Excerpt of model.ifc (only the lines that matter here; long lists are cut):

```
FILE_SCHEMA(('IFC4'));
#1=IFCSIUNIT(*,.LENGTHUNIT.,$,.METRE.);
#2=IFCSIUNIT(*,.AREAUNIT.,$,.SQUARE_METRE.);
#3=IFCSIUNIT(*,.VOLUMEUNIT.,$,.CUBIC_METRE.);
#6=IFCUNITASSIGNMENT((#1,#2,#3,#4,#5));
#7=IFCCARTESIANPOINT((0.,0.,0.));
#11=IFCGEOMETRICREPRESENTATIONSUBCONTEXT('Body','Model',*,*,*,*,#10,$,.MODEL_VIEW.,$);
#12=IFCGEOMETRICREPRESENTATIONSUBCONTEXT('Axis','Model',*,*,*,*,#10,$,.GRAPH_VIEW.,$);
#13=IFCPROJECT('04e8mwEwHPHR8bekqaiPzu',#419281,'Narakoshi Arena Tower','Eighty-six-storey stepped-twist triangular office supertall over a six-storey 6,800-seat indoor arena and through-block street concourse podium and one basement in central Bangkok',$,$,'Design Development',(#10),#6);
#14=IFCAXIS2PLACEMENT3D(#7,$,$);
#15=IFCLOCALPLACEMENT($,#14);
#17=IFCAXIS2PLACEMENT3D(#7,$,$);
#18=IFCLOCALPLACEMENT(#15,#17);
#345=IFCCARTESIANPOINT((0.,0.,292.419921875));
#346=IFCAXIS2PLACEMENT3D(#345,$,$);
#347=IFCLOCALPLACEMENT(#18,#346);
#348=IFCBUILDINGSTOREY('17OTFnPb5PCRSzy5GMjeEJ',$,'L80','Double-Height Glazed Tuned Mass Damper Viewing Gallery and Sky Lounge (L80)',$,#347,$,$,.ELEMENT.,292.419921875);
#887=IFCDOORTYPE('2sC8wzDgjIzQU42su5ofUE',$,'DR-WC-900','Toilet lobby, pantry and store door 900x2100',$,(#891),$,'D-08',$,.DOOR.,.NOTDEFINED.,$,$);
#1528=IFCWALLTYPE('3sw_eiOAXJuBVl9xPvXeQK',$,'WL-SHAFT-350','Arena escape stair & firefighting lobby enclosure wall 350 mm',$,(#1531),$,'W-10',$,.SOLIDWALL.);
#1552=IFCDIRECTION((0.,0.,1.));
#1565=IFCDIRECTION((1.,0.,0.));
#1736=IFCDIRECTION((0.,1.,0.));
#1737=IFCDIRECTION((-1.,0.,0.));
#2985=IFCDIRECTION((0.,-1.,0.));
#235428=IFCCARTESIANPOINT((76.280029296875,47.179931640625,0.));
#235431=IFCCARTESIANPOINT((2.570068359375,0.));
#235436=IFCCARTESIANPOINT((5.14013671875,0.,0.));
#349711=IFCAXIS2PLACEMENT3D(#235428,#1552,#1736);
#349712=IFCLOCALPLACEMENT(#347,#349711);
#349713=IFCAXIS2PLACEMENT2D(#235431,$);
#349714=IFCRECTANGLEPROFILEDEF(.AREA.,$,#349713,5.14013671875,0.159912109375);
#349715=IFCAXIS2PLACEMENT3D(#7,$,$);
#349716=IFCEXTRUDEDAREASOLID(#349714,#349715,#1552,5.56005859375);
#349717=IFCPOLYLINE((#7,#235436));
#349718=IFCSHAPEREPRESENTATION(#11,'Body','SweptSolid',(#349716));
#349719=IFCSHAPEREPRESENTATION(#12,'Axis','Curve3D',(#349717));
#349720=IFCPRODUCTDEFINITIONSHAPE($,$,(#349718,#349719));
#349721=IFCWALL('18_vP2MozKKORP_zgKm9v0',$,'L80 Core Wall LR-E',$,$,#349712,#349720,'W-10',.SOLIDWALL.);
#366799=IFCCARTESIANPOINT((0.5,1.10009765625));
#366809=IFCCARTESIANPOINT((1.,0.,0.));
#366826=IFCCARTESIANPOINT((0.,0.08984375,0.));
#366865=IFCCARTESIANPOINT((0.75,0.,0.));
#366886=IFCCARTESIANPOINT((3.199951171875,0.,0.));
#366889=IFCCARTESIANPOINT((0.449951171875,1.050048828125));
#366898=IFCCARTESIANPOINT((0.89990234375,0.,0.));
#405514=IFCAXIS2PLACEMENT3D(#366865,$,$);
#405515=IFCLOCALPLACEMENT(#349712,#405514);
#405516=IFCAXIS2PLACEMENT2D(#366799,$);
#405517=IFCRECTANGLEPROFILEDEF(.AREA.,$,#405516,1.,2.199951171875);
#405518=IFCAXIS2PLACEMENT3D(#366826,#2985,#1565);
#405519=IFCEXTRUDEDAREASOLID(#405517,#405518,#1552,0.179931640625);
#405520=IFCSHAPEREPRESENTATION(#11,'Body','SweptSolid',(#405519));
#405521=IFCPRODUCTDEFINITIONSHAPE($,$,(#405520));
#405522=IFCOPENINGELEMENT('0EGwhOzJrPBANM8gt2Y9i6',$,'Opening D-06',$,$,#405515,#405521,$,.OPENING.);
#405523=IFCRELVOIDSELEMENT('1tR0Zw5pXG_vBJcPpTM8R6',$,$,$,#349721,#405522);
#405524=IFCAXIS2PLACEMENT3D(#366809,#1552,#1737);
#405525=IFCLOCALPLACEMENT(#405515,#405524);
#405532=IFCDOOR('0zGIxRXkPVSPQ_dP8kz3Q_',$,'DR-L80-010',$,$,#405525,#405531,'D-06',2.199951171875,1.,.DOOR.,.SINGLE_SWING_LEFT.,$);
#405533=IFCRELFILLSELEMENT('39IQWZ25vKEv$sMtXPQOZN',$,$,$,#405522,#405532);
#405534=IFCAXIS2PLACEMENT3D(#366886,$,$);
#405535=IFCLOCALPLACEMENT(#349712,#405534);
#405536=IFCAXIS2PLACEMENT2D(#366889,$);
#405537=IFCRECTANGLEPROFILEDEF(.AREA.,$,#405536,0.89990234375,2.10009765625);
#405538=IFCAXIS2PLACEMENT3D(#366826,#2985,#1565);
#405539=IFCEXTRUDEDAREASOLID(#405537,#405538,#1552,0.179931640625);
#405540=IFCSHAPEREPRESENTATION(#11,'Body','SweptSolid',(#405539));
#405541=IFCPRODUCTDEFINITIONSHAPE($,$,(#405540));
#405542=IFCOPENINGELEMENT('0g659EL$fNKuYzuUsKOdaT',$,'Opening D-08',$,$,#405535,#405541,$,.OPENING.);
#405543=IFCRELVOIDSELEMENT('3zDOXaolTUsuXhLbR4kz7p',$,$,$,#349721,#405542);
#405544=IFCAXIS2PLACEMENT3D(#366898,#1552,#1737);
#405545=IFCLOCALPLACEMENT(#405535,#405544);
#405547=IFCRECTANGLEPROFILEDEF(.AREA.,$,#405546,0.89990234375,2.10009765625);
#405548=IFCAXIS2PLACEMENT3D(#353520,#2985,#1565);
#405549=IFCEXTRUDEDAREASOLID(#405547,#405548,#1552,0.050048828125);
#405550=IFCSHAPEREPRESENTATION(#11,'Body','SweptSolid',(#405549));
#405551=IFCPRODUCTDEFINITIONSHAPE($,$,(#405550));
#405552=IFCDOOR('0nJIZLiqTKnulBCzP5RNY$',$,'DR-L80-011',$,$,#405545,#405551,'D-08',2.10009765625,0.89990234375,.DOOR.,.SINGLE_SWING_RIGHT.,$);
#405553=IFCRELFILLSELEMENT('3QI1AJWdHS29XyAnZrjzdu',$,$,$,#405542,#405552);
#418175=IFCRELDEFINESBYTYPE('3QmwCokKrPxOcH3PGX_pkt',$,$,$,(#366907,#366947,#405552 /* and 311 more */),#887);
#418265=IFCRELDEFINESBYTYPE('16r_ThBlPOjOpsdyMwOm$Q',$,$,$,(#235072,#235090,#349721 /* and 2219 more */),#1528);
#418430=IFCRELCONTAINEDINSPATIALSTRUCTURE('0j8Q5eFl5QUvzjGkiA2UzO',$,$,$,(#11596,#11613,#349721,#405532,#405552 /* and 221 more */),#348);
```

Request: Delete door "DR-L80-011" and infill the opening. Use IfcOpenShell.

```python
import ifcopenshell
import ifcopenshell.api.feature
import ifcopenshell.api.root
import ifcopenshell.geom
import ifcopenshell.util.shape

model = ifcopenshell.open("model.ifc")
settings = ifcopenshell.geom.settings()


def volume(element):
    """Net volume in cubic metres, openings subtracted."""
    shape = ifcopenshell.geom.create_shape(settings, element)
    return ifcopenshell.util.shape.get_volume(shape.geometry)


door = model.by_guid("0nJIZLiqTKnulBCzP5RNY$")
opening = door.FillsVoids[0].RelatingOpeningElement
wall = opening.VoidsElements[0].RelatingBuildingElement
before = volume(wall)

ifcopenshell.api.root.remove_product(model, product=door)
ifcopenshell.api.feature.remove_feature(model, feature=opening)

after = volume(wall)

print(f"wall volume {before:.3f} -> {after:.3f} m3")

model.write("model_rev.ifc")
```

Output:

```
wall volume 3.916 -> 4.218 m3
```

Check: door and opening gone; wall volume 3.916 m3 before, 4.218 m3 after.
